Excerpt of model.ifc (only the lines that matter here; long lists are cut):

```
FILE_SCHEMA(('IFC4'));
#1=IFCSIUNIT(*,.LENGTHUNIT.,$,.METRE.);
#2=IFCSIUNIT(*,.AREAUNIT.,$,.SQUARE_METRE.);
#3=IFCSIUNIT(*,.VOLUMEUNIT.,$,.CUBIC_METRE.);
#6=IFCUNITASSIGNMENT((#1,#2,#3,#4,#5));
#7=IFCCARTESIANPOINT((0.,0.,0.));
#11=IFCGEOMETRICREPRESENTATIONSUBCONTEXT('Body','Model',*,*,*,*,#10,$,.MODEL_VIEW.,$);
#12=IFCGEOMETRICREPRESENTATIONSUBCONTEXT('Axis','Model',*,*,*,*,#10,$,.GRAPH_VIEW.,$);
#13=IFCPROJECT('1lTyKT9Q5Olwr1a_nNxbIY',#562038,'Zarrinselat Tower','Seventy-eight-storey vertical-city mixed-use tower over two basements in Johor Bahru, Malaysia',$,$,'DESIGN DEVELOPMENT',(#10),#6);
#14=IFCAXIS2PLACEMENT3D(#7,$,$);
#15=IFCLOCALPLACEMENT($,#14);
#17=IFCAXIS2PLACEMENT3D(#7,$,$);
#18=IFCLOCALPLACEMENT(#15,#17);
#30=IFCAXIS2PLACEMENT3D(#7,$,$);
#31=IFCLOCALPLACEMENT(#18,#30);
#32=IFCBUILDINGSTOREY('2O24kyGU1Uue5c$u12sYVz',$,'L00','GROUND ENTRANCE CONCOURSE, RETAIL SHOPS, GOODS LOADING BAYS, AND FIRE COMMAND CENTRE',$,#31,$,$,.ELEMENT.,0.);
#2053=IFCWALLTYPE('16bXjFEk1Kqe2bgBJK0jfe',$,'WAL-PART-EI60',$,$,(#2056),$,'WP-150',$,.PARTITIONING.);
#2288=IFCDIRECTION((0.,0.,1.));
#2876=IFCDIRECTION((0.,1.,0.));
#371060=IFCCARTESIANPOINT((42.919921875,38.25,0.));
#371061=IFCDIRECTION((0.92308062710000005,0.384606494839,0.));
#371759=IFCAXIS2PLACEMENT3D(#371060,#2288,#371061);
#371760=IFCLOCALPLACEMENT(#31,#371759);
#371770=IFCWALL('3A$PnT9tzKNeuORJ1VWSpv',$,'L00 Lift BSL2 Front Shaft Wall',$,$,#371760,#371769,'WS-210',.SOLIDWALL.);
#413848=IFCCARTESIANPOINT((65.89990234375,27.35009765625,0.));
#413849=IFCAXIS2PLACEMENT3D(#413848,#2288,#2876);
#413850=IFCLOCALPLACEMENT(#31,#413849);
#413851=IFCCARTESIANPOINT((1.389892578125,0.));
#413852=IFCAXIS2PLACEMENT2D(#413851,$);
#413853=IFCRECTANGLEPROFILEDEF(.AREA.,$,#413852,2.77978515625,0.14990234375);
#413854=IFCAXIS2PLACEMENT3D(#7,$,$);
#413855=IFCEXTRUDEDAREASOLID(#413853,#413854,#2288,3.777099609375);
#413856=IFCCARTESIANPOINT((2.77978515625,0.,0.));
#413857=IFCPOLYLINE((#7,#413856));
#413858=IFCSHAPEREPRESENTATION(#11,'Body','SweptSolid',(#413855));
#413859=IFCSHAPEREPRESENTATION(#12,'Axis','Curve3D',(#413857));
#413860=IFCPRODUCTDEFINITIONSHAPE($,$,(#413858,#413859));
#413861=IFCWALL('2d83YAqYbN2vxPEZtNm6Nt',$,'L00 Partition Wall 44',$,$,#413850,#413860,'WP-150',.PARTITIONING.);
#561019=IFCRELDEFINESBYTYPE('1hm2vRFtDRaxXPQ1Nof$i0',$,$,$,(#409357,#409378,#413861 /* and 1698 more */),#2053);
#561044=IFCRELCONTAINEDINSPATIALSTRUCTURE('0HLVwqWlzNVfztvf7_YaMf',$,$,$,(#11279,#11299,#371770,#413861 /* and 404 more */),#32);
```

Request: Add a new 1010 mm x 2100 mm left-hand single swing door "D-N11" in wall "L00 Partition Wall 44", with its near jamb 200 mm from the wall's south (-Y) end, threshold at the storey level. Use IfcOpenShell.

```python
import numpy as np
import ifcopenshell
import ifcopenshell.api.feature
import ifcopenshell.api.geometry
import ifcopenshell.api.root
import ifcopenshell.api.spatial
import ifcopenshell.geom
import ifcopenshell.util.element
import ifcopenshell.util.placement
import ifcopenshell.util.representation
import ifcopenshell.util.shape
import ifcopenshell.util.unit

model = ifcopenshell.open("model.ifc")
unit_scale = ifcopenshell.util.unit.calculate_unit_scale(model)
settings = ifcopenshell.geom.settings()


def volume(element):
    """Net volume in cubic metres, openings subtracted."""
    shape = ifcopenshell.geom.create_shape(settings, element)
    return ifcopenshell.util.shape.get_volume(shape.geometry)


wall = model.by_id(413861)
storey = ifcopenshell.util.element.get_container(wall, ifc_class="IfcBuildingStorey")
context = ifcopenshell.util.representation.get_context(model, "Model", "Body", "MODEL_VIEW")
before = volume(wall)

width, height, from_end, sill = 1.01, 2.1, 0.2, 0.0  # metres

# The wall runs along its own X axis, and the end named is its -X end.
wall_shape = ifcopenshell.geom.create_shape(settings, wall)
x, y, z = ifcopenshell.util.shape.get_vertices(wall_shape.geometry).T
start = x.min() + from_end
face, thickness = float(y.min()), float(y.max() - y.min())
wall_matrix = ifcopenshell.util.placement.get_local_placement(wall.ObjectPlacement)
level = ifcopenshell.util.placement.get_local_placement(storey.ObjectPlacement)[2, 3]


def in_wall(x, y):
    """Placement at x, y metres in the wall's axes, at sill height."""
    matrix = wall_matrix.copy()
    matrix[:, 3] = wall_matrix @ np.array([x / unit_scale, y / unit_scale, 0.0, 1.0])
    matrix[2, 3] = level + sill / unit_scale
    return matrix


# Opening: a box that overshoots both wall faces by 50 mm.
opening = ifcopenshell.api.root.create_entity(model, ifc_class="IfcOpeningElement", predefined_type="OPENING")
box = ifcopenshell.api.geometry.add_wall_representation(
    model, context=context, length=width, height=height, thickness=thickness + 0.1
)
ifcopenshell.api.geometry.assign_representation(model, product=opening, representation=box)
ifcopenshell.api.geometry.edit_object_placement(model, product=opening, matrix=in_wall(start, face - 0.05), is_si=False)
ifcopenshell.api.feature.add_feature(model, feature=opening, element=wall)

door = ifcopenshell.api.root.create_entity(model, ifc_class="IfcDoor", name="D-N11", predefined_type="DOOR")
door.OverallWidth, door.OverallHeight = width / unit_scale, height / unit_scale
door.OperationType = "SINGLE_SWING_LEFT"
body = ifcopenshell.api.geometry.add_door_representation(
    model,
    context=context,
    overall_width=door.OverallWidth,
    overall_height=door.OverallHeight,
    operation_type="SINGLE_SWING_LEFT",
    lining_properties={"LiningDepth": thickness / unit_scale, "ThresholdDepth": thickness / unit_scale},
)
ifcopenshell.api.geometry.assign_representation(model, product=door, representation=body)
ifcopenshell.api.spatial.assign_container(model, products=[door], relating_structure=storey)
ifcopenshell.api.feature.add_filling(model, opening=opening, element=door)

# The lining spans the wall, so the door starts at the wall face.
ifcopenshell.api.geometry.edit_object_placement(model, product=door, matrix=in_wall(start, face), is_si=False)

after = volume(wall)

print(f"wall volume {before:.3f} -> {after:.3f} m3")

model.write("model_edited.ifc")
```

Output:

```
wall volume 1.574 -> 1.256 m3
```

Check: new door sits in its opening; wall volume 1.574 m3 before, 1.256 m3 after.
